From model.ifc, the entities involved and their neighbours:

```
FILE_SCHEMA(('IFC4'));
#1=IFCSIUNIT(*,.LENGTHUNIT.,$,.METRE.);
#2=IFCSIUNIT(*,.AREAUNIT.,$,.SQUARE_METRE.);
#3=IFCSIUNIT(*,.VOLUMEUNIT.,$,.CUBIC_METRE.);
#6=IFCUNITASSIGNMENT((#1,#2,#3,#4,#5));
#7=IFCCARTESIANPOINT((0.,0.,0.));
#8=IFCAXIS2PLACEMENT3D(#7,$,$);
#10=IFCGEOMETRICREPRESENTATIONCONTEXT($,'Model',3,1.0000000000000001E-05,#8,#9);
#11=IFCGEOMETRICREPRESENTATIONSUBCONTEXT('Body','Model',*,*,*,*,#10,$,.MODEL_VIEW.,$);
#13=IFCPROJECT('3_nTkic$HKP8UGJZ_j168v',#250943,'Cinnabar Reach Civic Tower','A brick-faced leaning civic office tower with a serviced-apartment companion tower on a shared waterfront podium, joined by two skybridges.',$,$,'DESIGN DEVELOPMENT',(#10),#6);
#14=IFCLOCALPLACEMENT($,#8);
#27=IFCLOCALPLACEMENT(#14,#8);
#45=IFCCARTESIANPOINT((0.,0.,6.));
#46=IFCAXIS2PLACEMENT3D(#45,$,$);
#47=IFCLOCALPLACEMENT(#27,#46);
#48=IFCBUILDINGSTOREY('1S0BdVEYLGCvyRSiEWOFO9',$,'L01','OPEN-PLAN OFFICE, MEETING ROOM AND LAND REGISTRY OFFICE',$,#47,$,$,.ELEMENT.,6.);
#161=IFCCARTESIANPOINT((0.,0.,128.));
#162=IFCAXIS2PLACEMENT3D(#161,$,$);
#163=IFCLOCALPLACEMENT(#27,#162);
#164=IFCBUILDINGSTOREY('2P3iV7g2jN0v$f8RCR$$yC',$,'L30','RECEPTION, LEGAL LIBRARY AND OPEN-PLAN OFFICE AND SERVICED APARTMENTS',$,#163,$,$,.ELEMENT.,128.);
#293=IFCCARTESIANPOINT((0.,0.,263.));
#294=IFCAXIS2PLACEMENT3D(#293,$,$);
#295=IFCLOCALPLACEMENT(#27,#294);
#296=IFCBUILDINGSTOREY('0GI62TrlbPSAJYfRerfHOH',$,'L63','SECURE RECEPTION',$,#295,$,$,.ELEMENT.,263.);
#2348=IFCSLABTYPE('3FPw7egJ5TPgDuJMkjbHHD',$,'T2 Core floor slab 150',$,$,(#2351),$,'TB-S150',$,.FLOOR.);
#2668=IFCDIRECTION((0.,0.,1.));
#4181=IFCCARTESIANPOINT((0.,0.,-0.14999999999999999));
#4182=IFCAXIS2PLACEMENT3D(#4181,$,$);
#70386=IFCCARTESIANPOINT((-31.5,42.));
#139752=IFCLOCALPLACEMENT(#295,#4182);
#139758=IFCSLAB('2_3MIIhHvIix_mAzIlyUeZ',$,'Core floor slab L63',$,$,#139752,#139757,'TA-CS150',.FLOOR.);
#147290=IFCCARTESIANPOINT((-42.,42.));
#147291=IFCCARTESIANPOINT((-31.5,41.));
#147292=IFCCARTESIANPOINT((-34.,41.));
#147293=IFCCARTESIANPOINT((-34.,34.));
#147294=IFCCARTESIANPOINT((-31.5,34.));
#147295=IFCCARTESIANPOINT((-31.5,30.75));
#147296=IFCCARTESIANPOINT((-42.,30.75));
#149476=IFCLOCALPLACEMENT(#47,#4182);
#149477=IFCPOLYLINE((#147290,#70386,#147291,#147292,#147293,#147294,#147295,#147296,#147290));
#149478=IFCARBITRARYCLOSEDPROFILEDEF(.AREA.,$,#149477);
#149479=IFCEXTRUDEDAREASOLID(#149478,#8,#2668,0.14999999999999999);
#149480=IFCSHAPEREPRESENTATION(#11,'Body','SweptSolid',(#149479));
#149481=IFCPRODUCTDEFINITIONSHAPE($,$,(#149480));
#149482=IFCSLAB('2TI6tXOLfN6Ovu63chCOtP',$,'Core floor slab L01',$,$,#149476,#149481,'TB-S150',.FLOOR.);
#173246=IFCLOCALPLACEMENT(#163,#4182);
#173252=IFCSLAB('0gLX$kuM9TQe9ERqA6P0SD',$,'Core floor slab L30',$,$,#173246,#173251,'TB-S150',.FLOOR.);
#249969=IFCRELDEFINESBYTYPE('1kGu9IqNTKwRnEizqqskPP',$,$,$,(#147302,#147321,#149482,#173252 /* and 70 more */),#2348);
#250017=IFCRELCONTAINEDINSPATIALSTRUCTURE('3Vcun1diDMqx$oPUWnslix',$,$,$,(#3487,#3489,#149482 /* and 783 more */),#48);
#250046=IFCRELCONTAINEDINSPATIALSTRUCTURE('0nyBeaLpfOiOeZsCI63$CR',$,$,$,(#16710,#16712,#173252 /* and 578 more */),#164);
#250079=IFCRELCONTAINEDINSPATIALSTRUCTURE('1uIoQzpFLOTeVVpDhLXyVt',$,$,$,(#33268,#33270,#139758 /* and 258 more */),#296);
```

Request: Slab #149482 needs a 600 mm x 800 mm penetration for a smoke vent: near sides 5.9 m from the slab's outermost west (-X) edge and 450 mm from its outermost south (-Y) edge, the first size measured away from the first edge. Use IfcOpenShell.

```python
import numpy as np
import ifcopenshell
import ifcopenshell.api.feature
import ifcopenshell.api.geometry
import ifcopenshell.api.root
import ifcopenshell.geom
import ifcopenshell.util.placement
import ifcopenshell.util.representation
import ifcopenshell.util.shape
import ifcopenshell.util.unit

model = ifcopenshell.open("model.ifc")
unit_scale = ifcopenshell.util.unit.calculate_unit_scale(model)
settings = ifcopenshell.geom.settings()


def volume(element):
    """Net volume in cubic metres, openings subtracted."""
    shape = ifcopenshell.geom.create_shape(settings, element)
    return ifcopenshell.util.shape.get_volume(shape.geometry)


slab = model.by_guid("2TI6tXOLfN6Ovu63chCOtP")
before = volume(slab)

# Extent in the slab's own axes, in metres. The edges named are its -X and -Y sides.
slab_shape = ifcopenshell.geom.create_shape(settings, slab)
vertices = ifcopenshell.util.shape.get_vertices(slab_shape.geometry)
x_min, y_min, bottom = vertices.min(axis=0)
top = vertices[:, 2].max()

opening = ifcopenshell.api.root.create_entity(model, ifc_class="IfcOpeningElement", name="Smoke vent opening", predefined_type="OPENING")
context = ifcopenshell.util.representation.get_context(model, "Model", "Body", "MODEL_VIEW")
width, depth = 0.6, 0.8
outline = [(0.0, 0.0), (width, 0.0), (width, depth), (0.0, depth), (0.0, 0.0)]
# Overshoot both faces by 50 mm so the cut is clean.
shape = ifcopenshell.api.geometry.add_slab_representation(
    model, context=context, depth=top - bottom + 0.1, polyline=outline
)
ifcopenshell.api.geometry.assign_representation(model, product=opening, representation=shape)

matrix = ifcopenshell.util.placement.get_local_placement(slab.ObjectPlacement)
matrix[:, 3] = matrix @ np.append(np.array([x_min + 5.9, y_min + 0.45, bottom - 0.05]) / unit_scale, 1.0)
ifcopenshell.api.geometry.edit_object_placement(model, product=opening, matrix=matrix, is_si=False)
ifcopenshell.api.feature.add_feature(model, feature=opening, element=slab)

after = volume(slab)

print(f"slab volume {before:.3f} -> {after:.3f} m3")

model.write("model_rev.ifc")
```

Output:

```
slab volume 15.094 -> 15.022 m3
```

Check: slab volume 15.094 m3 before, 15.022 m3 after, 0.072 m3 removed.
